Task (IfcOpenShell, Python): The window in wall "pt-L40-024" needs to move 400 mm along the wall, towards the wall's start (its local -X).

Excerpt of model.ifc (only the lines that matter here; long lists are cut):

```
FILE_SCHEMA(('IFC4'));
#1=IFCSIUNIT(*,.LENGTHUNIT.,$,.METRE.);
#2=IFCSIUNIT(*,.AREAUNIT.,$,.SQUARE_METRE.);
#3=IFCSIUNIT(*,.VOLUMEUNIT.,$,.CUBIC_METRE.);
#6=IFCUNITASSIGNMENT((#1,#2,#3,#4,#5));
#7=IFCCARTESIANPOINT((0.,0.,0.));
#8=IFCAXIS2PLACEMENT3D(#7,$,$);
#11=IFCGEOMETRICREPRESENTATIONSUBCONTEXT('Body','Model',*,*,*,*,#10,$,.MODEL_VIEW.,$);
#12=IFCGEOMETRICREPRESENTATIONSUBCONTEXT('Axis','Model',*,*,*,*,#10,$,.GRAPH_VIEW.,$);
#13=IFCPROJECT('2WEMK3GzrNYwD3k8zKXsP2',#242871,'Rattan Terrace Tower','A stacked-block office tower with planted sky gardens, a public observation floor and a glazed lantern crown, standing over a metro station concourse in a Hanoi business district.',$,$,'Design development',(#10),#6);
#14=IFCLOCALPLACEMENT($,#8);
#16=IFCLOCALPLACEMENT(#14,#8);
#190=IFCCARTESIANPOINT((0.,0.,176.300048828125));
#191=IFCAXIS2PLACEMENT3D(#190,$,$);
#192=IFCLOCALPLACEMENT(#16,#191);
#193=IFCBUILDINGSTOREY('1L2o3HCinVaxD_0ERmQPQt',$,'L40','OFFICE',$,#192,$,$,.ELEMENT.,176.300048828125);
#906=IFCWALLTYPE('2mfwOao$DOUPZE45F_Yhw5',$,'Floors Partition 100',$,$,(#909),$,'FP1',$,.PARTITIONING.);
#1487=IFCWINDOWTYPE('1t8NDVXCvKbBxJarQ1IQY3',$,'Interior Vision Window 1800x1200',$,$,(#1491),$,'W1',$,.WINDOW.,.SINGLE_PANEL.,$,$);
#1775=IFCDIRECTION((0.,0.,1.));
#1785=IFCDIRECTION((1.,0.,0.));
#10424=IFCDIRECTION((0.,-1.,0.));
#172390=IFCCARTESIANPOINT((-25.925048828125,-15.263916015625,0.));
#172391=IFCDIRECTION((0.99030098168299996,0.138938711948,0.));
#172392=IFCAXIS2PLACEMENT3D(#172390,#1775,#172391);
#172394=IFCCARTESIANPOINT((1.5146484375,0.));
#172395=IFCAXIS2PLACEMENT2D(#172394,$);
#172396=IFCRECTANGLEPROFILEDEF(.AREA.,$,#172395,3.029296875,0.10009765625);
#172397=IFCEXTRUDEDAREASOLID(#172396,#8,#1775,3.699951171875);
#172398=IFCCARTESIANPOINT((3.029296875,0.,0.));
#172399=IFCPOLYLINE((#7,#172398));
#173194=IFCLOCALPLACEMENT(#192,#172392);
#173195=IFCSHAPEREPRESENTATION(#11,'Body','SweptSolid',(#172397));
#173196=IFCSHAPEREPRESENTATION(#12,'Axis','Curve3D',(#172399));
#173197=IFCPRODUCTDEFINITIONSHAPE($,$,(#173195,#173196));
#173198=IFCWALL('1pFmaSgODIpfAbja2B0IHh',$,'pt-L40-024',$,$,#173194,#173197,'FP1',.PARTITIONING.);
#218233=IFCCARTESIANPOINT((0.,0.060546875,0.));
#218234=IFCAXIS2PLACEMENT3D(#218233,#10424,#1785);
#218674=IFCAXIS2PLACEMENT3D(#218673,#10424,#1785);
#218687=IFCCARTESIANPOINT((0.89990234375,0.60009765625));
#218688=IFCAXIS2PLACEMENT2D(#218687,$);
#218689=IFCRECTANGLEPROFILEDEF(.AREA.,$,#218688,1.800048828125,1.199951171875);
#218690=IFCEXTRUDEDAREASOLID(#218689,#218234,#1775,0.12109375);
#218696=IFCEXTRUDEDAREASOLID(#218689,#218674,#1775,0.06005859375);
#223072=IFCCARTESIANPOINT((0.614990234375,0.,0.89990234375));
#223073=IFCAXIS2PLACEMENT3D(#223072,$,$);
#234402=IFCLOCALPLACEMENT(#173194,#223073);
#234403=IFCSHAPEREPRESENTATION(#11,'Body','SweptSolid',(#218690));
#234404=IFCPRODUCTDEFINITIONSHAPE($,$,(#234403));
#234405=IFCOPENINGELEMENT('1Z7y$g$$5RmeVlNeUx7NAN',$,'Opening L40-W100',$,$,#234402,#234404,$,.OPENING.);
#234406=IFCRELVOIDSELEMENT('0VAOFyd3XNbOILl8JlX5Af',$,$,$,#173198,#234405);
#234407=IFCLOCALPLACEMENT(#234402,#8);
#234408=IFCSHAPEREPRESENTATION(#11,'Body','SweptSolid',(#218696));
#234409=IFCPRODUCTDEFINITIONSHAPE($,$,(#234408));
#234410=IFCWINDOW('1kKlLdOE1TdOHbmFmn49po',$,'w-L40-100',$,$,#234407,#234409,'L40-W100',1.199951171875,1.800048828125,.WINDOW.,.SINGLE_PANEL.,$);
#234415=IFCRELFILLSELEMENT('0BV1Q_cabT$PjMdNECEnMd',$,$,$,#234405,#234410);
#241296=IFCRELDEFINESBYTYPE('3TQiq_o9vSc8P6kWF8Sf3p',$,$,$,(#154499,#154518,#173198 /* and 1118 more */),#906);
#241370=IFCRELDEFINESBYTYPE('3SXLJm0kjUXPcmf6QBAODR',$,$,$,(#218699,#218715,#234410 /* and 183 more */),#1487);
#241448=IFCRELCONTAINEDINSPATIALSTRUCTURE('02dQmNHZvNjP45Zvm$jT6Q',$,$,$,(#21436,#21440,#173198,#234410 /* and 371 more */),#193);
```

```python
import ifcopenshell
import ifcopenshell.api.geometry
import ifcopenshell.util.placement

model = ifcopenshell.open("model.ifc")

window = model.by_id(234410)
opening = window.FillsVoids[0].RelatingOpeningElement
wall = opening.VoidsElements[0].RelatingBuildingElement

wall_matrix = ifcopenshell.util.placement.get_local_placement(wall.ObjectPlacement)
shift = wall_matrix[:3, 0] * -0.4
before = ifcopenshell.util.placement.get_local_placement(window.ObjectPlacement)[:3, 3].copy()

# The window is placed relative to its opening, so it follows when the opening moves.
matrix = ifcopenshell.util.placement.get_local_placement(opening.ObjectPlacement)
matrix[:3, 3] += shift
ifcopenshell.api.geometry.edit_object_placement(
    model, product=opening, matrix=matrix, is_si=False, should_transform_children=True
)

after = ifcopenshell.util.placement.get_local_placement(window.ObjectPlacement)[:3, 3]
print("window moved by", (after - before).round(3) + 0.0)

model.write("model_rev.ifc")
```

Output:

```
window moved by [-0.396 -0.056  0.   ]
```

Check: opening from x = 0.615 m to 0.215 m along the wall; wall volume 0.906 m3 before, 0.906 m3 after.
